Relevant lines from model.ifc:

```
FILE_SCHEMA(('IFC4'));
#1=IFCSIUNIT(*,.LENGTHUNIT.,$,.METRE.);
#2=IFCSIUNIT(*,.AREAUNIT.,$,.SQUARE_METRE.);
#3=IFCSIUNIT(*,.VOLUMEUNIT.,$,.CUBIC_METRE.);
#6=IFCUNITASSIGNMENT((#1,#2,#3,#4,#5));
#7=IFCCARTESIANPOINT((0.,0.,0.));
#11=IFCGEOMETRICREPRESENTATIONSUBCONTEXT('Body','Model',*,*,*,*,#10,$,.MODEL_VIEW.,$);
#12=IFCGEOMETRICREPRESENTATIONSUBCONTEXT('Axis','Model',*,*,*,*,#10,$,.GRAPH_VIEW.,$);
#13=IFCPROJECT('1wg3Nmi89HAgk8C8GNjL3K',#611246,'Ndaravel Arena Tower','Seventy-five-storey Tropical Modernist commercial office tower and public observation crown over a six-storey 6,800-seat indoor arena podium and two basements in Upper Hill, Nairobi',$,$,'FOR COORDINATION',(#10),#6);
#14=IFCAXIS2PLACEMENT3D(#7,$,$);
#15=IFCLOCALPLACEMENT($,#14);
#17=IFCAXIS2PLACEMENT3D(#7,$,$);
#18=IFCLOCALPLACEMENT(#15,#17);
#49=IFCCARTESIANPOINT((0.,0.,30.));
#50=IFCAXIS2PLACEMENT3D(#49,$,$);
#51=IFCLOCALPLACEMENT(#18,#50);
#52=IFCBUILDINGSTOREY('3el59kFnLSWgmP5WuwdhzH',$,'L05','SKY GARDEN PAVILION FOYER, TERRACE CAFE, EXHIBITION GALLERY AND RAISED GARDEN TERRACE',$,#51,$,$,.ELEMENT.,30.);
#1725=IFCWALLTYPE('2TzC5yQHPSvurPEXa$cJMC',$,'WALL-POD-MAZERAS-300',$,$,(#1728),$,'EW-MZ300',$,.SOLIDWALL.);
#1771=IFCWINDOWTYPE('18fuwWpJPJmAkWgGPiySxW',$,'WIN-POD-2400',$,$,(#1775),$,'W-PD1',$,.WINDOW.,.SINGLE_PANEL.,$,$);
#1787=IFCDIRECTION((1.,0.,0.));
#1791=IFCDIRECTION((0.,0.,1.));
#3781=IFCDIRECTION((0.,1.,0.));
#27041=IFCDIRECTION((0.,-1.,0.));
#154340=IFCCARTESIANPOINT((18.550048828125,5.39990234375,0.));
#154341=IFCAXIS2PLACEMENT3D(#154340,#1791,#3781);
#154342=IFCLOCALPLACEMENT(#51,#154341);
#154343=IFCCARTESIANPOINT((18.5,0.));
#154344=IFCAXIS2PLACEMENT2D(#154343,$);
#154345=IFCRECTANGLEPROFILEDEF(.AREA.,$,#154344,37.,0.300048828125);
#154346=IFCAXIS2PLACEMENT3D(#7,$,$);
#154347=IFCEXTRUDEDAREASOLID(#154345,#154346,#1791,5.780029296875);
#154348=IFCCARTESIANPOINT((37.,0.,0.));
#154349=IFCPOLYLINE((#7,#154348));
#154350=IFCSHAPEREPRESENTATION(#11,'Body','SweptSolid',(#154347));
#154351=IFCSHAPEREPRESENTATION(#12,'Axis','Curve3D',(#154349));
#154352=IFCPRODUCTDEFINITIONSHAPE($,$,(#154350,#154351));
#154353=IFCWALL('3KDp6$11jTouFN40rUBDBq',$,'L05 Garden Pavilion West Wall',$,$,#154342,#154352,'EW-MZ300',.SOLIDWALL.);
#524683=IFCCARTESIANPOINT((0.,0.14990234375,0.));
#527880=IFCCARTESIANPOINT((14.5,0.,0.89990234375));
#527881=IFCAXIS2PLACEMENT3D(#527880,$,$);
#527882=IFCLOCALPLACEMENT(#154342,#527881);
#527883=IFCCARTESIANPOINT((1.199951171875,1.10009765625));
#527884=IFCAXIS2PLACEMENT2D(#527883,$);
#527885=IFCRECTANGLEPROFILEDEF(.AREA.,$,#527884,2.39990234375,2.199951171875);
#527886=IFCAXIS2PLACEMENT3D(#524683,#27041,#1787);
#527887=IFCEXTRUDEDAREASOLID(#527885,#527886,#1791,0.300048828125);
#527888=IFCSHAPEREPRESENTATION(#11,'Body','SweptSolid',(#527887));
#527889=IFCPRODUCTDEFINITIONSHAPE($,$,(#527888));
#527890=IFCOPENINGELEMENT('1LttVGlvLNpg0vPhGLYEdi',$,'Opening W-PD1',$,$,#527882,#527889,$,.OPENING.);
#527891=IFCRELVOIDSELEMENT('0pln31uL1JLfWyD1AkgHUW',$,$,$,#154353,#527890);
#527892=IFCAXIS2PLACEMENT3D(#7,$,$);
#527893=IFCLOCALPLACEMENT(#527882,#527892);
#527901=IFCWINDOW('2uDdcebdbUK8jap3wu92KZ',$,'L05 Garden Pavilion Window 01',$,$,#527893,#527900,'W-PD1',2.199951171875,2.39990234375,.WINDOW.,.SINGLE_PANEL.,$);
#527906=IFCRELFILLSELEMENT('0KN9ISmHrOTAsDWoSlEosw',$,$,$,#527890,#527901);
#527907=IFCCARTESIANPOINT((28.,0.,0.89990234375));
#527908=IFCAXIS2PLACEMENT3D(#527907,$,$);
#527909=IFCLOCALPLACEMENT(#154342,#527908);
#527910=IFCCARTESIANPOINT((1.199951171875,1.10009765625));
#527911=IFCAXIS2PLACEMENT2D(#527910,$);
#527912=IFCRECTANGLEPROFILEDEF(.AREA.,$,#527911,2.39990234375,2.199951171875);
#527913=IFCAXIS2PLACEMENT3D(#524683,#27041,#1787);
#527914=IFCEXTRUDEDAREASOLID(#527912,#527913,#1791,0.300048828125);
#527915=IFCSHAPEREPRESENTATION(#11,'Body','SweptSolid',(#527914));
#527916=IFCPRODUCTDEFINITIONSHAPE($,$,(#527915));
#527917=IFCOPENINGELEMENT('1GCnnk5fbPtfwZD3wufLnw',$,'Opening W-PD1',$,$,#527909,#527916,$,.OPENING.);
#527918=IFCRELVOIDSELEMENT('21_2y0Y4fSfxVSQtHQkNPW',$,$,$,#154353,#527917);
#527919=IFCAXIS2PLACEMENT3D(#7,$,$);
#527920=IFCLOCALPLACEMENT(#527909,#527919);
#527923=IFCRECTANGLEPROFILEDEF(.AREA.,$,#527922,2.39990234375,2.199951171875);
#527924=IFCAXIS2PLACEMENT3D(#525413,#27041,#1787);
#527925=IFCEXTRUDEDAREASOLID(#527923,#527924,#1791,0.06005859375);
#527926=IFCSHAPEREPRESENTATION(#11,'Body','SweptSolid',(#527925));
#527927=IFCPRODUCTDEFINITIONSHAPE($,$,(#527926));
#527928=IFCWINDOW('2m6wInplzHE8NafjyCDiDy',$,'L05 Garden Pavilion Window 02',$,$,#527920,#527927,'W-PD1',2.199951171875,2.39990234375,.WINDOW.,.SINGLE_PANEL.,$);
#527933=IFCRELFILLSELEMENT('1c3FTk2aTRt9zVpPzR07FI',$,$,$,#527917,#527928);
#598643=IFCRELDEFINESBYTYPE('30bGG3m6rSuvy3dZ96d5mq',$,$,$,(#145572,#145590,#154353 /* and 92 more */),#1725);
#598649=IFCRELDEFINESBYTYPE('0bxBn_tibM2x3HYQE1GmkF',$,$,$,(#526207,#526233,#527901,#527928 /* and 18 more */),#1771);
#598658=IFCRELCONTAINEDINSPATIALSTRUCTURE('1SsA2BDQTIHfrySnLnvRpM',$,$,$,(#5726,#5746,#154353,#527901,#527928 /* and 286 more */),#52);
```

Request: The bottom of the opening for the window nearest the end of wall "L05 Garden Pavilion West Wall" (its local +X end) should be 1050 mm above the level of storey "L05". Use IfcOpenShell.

```python
import numpy as np
import ifcopenshell
import ifcopenshell.api.geometry
import ifcopenshell.geom
import ifcopenshell.util.element
import ifcopenshell.util.placement
import ifcopenshell.util.shape
import ifcopenshell.util.unit

model = ifcopenshell.open("model.ifc")
unit_scale = ifcopenshell.util.unit.calculate_unit_scale(model)

window = model.by_guid("2m6wInplzHE8NafjyCDiDy")
opening = window.FillsVoids[0].RelatingOpeningElement
storey = ifcopenshell.util.element.get_container(window, ifc_class="IfcBuildingStorey")
level = ifcopenshell.util.placement.get_local_placement(storey.ObjectPlacement)[2, 3]

# The opening's origin need not be at the sill, so measure its lowest point.
shape = ifcopenshell.geom.create_shape(ifcopenshell.geom.settings(), opening)
bottom = ifcopenshell.util.shape.get_shape_bottom_elevation(shape, shape.geometry) / unit_scale
dz = level + 1.05 / unit_scale - bottom

shift = np.array([0.0, 0.0, dz])
# The window is placed relative to its opening, so it follows when the opening moves.
matrix = ifcopenshell.util.placement.get_local_placement(opening.ObjectPlacement)
matrix[:3, 3] += shift
ifcopenshell.api.geometry.edit_object_placement(
    model, product=opening, matrix=matrix, is_si=False, should_transform_children=True
)

print(f"moved by {dz * unit_scale:+.3f} m")

model.write("model-out.ifc")
```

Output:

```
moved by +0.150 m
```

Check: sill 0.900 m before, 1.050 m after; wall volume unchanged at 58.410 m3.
